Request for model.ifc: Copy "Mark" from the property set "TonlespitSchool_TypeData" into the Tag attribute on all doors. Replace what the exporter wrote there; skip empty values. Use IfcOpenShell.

First a look at what the model holds.

```python
import ifcopenshell
import ifcopenshell.util.element

model = ifcopenshell.open("model.ifc")
print(model.schema)
doors = model.by_type("IfcDoor")
print(len(doors), "doors")
for e in doors[:8]:
    source = ifcopenshell.util.element.get_pset(e, "TonlespitSchool_TypeData", "Mark")
    target = e.Tag
    print(e.id(), repr(source), repr(target), sep=" | ")
```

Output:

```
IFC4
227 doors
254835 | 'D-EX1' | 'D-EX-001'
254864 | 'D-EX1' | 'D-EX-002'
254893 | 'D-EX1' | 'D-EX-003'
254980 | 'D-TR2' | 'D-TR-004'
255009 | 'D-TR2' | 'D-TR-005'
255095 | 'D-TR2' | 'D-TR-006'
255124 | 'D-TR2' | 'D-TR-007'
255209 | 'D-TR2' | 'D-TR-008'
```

```python
import ifcopenshell
import ifcopenshell.util.element

model = ifcopenshell.open("model.ifc")

count = 0
for e in model.by_type("IfcDoor"):
    value = ifcopenshell.util.element.get_pset(e, "TonlespitSchool_TypeData", "Mark")
    current = e.Tag
    if not value or not value.strip() or current == value:
        continue
    e.Tag = value
    count += 1

print(count, "doors updated")

model.write("model_edited.ifc")
```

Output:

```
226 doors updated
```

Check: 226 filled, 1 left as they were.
